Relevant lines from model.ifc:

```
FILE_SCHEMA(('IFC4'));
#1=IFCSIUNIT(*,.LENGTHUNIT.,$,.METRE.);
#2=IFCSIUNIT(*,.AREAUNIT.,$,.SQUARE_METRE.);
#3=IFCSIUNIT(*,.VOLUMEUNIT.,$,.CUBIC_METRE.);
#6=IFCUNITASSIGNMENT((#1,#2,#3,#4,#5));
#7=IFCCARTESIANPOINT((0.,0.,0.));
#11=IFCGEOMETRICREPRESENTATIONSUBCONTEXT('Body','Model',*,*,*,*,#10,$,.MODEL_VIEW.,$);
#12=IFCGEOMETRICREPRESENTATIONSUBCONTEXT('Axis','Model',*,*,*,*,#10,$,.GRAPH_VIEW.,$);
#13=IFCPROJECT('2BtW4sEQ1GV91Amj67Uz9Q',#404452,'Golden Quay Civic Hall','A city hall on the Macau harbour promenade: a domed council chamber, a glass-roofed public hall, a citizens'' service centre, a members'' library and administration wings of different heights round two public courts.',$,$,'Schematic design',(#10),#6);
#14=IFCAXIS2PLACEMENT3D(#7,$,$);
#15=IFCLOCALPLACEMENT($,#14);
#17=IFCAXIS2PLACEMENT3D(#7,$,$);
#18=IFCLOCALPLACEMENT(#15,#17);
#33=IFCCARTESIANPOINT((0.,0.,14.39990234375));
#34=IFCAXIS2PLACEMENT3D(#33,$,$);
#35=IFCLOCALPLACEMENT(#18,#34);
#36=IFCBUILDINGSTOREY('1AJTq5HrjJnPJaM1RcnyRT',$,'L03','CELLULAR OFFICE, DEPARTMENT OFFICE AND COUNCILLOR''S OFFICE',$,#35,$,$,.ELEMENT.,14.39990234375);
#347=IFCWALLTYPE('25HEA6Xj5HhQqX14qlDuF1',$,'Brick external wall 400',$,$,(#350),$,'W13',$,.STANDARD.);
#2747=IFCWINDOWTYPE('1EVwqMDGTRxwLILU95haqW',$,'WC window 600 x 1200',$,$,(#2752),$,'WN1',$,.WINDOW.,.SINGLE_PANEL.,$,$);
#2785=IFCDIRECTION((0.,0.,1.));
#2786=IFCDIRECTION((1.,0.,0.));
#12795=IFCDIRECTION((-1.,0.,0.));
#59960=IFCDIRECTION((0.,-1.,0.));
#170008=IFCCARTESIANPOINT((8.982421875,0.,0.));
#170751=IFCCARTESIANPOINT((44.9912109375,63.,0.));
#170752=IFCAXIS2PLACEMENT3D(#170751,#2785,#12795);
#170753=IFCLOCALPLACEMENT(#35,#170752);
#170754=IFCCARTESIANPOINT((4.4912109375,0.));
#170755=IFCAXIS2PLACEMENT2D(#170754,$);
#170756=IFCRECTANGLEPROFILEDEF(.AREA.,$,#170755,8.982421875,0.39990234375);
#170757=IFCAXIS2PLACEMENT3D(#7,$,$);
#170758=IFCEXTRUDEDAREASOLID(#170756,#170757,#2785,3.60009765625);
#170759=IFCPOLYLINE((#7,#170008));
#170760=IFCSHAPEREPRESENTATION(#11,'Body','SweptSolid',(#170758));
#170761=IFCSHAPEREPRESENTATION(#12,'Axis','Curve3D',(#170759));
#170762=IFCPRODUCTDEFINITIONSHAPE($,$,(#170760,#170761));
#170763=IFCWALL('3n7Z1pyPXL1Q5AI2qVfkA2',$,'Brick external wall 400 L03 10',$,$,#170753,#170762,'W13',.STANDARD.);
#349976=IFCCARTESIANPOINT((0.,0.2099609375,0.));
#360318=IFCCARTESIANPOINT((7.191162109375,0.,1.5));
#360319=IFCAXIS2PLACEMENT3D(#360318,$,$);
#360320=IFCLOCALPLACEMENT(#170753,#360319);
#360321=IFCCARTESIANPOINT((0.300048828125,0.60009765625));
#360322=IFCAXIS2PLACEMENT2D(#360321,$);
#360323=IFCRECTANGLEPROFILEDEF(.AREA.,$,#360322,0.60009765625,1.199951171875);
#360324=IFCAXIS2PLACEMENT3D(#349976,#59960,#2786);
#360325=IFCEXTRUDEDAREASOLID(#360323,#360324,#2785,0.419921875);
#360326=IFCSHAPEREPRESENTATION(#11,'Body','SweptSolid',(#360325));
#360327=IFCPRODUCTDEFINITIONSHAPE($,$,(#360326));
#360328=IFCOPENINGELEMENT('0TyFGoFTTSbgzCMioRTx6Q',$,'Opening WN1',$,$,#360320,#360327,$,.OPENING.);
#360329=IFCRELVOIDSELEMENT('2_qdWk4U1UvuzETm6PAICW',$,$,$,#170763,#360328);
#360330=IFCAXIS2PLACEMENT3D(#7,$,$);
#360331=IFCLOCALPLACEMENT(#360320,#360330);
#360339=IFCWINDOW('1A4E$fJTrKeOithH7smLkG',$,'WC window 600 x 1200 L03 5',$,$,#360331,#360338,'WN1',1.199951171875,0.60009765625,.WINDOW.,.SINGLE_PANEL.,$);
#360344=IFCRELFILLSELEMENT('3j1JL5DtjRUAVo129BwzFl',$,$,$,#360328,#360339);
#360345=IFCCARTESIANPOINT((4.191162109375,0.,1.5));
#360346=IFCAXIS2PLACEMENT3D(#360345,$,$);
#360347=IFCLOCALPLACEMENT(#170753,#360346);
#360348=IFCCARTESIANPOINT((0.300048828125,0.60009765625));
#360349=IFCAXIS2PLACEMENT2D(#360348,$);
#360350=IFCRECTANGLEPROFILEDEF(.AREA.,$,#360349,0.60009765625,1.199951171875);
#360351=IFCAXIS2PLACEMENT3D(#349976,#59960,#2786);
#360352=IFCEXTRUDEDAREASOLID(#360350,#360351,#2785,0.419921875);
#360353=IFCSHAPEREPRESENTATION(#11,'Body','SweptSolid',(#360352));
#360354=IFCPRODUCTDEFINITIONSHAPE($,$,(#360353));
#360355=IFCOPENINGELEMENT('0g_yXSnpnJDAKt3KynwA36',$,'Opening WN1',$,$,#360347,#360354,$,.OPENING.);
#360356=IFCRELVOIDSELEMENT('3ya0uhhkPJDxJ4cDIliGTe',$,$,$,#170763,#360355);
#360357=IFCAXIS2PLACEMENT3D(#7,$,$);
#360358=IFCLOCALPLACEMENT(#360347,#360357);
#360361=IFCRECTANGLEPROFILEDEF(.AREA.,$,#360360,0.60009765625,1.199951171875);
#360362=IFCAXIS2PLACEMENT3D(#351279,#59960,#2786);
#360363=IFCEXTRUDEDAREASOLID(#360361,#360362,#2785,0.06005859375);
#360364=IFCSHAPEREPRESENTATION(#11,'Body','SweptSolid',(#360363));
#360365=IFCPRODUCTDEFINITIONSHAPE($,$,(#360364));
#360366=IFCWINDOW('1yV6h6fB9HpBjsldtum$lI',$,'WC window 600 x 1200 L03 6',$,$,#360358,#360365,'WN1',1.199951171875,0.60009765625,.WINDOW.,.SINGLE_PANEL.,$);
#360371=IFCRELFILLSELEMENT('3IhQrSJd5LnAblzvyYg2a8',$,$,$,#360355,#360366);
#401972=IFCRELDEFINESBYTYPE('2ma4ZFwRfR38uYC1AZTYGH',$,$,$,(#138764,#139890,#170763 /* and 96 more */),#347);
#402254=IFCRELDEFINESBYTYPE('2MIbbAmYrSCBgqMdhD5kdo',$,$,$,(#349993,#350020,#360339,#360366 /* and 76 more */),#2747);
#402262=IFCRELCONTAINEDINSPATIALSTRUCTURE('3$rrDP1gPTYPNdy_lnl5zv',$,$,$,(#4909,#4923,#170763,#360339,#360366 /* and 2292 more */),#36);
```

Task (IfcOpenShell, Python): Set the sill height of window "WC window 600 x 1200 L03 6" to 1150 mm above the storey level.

```python
import numpy as np
import ifcopenshell
import ifcopenshell.api.geometry
import ifcopenshell.geom
import ifcopenshell.util.element
import ifcopenshell.util.placement
import ifcopenshell.util.shape
import ifcopenshell.util.unit

model = ifcopenshell.open("model.ifc")
unit_scale = ifcopenshell.util.unit.calculate_unit_scale(model)

window = model.by_id(360366)
opening = window.FillsVoids[0].RelatingOpeningElement
storey = ifcopenshell.util.element.get_container(window, ifc_class="IfcBuildingStorey")
level = ifcopenshell.util.placement.get_local_placement(storey.ObjectPlacement)[2, 3]

# The opening's origin need not be at the sill, so measure its lowest point.
shape = ifcopenshell.geom.create_shape(ifcopenshell.geom.settings(), opening)
bottom = ifcopenshell.util.shape.get_shape_bottom_elevation(shape, shape.geometry) / unit_scale
dz = level + 1.15 / unit_scale - bottom

shift = np.array([0.0, 0.0, dz])
# The window is placed relative to its opening, so it follows when the opening moves.
matrix = ifcopenshell.util.placement.get_local_placement(opening.ObjectPlacement)
matrix[:3, 3] += shift
ifcopenshell.api.geometry.edit_object_placement(
    model, product=opening, matrix=matrix, is_si=False, should_transform_children=True
)

print(f"moved by {dz * unit_scale:+.3f} m")

model.write("model_updated.ifc")
```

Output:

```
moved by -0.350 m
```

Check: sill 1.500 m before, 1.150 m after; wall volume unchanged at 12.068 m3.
